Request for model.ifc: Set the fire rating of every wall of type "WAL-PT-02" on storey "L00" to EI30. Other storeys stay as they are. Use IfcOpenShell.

First a look at what the model holds.

```python
import ifcopenshell
import ifcopenshell.util.element

model = ifcopenshell.open("model.ifc")
print(model.schema)
storey = next(s for s in model.by_type("IfcBuildingStorey") if s.Name == "L00")
walls = [e for e in ifcopenshell.util.element.get_decomposition(storey) if e.is_a("IfcWall")]
seen = {}
for e in walls:
    element_type = ifcopenshell.util.element.get_type(e)
    key = (element_type.Name if element_type != e and element_type else None, ifcopenshell.util.element.get_pset(e, "Pset_WallCommon", "FireRating"))
    seen[key] = seen.get(key, 0) + 1
for (name, value), count in sorted(seen.items(), key=str):
    print(count, "x", name, "|", value)
```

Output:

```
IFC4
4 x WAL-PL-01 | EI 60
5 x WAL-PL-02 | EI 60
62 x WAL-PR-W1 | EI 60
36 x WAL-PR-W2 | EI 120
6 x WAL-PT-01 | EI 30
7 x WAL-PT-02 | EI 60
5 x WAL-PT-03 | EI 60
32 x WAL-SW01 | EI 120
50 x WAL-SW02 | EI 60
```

```python
import ifcopenshell
import ifcopenshell.api.pset
import ifcopenshell.util.element

model = ifcopenshell.open("model.ifc")

storey = next(s for s in model.by_type("IfcBuildingStorey") if s.Name == "L00")
walls = [e for e in ifcopenshell.util.element.get_decomposition(storey) if e.is_a("IfcWall")]

count = 0
for e in walls:
    element_type = ifcopenshell.util.element.get_type(e)
    if element_type in (None, e) or element_type.Name != "WAL-PT-02":
        continue
    # add_pset returns the element's existing set when there is one.
    pset = ifcopenshell.api.pset.add_pset(model, product=e, name="Pset_WallCommon")
    ifcopenshell.api.pset.edit_pset(model, pset=pset, properties={"FireRating": "EI30"})
    count += 1

print(count, "walls updated")

model.write("model_v2.ifc")
```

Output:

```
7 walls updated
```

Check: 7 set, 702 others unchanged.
